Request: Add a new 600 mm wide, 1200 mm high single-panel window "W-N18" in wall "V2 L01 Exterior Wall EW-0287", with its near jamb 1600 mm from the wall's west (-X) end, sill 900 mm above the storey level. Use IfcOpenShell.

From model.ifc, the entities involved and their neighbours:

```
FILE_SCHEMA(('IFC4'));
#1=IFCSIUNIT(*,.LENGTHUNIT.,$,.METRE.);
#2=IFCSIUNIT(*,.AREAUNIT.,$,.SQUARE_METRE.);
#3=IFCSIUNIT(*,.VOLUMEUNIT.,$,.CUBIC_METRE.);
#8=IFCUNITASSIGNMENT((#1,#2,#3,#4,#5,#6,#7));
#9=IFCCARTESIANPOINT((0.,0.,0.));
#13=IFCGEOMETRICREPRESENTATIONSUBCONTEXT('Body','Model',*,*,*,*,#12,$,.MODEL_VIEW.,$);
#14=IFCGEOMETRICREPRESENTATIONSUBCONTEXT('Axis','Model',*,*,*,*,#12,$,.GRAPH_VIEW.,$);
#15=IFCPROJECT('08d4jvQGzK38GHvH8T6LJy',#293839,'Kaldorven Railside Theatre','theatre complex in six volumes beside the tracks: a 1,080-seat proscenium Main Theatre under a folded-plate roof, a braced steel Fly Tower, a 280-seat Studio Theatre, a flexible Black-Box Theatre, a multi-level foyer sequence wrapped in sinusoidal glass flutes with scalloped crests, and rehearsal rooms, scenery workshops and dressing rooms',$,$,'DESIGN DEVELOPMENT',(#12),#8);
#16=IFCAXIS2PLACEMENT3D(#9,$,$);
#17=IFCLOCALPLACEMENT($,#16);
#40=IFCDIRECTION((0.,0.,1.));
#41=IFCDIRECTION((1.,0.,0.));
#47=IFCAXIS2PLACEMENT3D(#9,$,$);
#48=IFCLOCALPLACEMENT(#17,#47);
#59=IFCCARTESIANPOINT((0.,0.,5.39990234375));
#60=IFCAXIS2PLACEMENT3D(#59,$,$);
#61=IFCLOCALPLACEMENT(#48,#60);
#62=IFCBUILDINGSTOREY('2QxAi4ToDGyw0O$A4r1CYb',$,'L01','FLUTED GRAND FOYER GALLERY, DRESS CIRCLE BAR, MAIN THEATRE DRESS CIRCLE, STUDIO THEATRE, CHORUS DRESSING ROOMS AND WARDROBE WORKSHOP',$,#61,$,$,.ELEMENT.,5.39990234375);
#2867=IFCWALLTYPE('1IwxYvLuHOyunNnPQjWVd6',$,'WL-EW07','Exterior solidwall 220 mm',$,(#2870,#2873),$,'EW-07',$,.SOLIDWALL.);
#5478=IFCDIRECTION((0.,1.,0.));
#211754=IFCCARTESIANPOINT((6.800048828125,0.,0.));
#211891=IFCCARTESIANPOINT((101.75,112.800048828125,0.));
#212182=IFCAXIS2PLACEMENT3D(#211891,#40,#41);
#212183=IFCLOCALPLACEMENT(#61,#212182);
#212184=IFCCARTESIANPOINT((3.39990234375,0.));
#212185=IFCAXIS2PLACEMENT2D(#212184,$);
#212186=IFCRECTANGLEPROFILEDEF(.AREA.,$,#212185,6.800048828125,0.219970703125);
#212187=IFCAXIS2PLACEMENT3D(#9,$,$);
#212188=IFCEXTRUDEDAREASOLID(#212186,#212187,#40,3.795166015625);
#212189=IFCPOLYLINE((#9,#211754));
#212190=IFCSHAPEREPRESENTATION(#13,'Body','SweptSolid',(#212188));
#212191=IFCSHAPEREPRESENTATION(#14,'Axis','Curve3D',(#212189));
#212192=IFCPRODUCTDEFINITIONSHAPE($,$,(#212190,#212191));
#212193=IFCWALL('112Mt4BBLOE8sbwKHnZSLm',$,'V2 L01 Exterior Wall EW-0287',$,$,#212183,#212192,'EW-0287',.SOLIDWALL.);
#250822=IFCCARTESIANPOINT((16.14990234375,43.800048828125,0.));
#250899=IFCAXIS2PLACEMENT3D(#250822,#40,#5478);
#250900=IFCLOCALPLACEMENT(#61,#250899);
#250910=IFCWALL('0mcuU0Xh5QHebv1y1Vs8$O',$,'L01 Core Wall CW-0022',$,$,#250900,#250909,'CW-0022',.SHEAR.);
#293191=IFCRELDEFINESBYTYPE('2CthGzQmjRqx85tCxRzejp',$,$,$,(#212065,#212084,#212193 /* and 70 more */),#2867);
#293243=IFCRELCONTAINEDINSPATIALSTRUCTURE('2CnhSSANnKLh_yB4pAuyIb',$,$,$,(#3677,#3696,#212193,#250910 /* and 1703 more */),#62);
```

```python
import numpy as np
import ifcopenshell
import ifcopenshell.api.feature
import ifcopenshell.api.geometry
import ifcopenshell.api.root
import ifcopenshell.api.spatial
import ifcopenshell.geom
import ifcopenshell.util.element
import ifcopenshell.util.placement
import ifcopenshell.util.representation
import ifcopenshell.util.shape
import ifcopenshell.util.unit

model = ifcopenshell.open("model.ifc")
unit_scale = ifcopenshell.util.unit.calculate_unit_scale(model)
settings = ifcopenshell.geom.settings()


def volume(element):
    """Net volume in cubic metres, openings subtracted."""
    shape = ifcopenshell.geom.create_shape(settings, element)
    return ifcopenshell.util.shape.get_volume(shape.geometry)


wall = model.by_id(212193)
storey = ifcopenshell.util.element.get_container(wall, ifc_class="IfcBuildingStorey")
context = ifcopenshell.util.representation.get_context(model, "Model", "Body", "MODEL_VIEW")
before = volume(wall)

width, height, from_end, sill = 0.6, 1.2, 1.6, 0.9  # metres

# The wall runs along its own X axis, and the end named is its -X end.
wall_shape = ifcopenshell.geom.create_shape(settings, wall)
x, y, z = ifcopenshell.util.shape.get_vertices(wall_shape.geometry).T
start = x.min() + from_end
face, thickness = float(y.min()), float(y.max() - y.min())
wall_matrix = ifcopenshell.util.placement.get_local_placement(wall.ObjectPlacement)
level = ifcopenshell.util.placement.get_local_placement(storey.ObjectPlacement)[2, 3]


def in_wall(x, y):
    """Placement at x, y metres in the wall's axes, at sill height."""
    matrix = wall_matrix.copy()
    matrix[:, 3] = wall_matrix @ np.array([x / unit_scale, y / unit_scale, 0.0, 1.0])
    matrix[2, 3] = level + sill / unit_scale
    return matrix


# Opening: a box that overshoots both wall faces by 50 mm.
opening = ifcopenshell.api.root.create_entity(model, ifc_class="IfcOpeningElement", predefined_type="OPENING")
box = ifcopenshell.api.geometry.add_wall_representation(
    model, context=context, length=width, height=height, thickness=thickness + 0.1
)
ifcopenshell.api.geometry.assign_representation(model, product=opening, representation=box)
ifcopenshell.api.geometry.edit_object_placement(model, product=opening, matrix=in_wall(start, face - 0.05), is_si=False)
ifcopenshell.api.feature.add_feature(model, feature=opening, element=wall)

window = ifcopenshell.api.root.create_entity(model, ifc_class="IfcWindow", name="W-N18", predefined_type="WINDOW")
window.OverallWidth, window.OverallHeight = width / unit_scale, height / unit_scale
window.PartitioningType = "SINGLE_PANEL"
body = ifcopenshell.api.geometry.add_window_representation(
    model,
    context=context,
    overall_width=window.OverallWidth,
    overall_height=window.OverallHeight,
    partition_type="SINGLE_PANEL",
)
ifcopenshell.api.geometry.assign_representation(model, product=window, representation=body)
ifcopenshell.api.spatial.assign_container(model, products=[window], relating_structure=storey)
ifcopenshell.api.feature.add_filling(model, opening=opening, element=window)

# Centre the window in the wall's thickness.
ifcopenshell.api.geometry.edit_object_placement(model, product=window, matrix=in_wall(start, face), is_si=False)
window_shape = ifcopenshell.geom.create_shape(settings, window)
depth = ifcopenshell.util.shape.get_vertices(window_shape.geometry)[:, 1]
offset = face + thickness / 2 - (depth.min() + depth.max()) / 2
ifcopenshell.api.geometry.edit_object_placement(model, product=window, matrix=in_wall(start, offset), is_si=False)

after = volume(wall)

print(f"wall volume {before:.3f} -> {after:.3f} m3")

model.write("model-out.ifc")
```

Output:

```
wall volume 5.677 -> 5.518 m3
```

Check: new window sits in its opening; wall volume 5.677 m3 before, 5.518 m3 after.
